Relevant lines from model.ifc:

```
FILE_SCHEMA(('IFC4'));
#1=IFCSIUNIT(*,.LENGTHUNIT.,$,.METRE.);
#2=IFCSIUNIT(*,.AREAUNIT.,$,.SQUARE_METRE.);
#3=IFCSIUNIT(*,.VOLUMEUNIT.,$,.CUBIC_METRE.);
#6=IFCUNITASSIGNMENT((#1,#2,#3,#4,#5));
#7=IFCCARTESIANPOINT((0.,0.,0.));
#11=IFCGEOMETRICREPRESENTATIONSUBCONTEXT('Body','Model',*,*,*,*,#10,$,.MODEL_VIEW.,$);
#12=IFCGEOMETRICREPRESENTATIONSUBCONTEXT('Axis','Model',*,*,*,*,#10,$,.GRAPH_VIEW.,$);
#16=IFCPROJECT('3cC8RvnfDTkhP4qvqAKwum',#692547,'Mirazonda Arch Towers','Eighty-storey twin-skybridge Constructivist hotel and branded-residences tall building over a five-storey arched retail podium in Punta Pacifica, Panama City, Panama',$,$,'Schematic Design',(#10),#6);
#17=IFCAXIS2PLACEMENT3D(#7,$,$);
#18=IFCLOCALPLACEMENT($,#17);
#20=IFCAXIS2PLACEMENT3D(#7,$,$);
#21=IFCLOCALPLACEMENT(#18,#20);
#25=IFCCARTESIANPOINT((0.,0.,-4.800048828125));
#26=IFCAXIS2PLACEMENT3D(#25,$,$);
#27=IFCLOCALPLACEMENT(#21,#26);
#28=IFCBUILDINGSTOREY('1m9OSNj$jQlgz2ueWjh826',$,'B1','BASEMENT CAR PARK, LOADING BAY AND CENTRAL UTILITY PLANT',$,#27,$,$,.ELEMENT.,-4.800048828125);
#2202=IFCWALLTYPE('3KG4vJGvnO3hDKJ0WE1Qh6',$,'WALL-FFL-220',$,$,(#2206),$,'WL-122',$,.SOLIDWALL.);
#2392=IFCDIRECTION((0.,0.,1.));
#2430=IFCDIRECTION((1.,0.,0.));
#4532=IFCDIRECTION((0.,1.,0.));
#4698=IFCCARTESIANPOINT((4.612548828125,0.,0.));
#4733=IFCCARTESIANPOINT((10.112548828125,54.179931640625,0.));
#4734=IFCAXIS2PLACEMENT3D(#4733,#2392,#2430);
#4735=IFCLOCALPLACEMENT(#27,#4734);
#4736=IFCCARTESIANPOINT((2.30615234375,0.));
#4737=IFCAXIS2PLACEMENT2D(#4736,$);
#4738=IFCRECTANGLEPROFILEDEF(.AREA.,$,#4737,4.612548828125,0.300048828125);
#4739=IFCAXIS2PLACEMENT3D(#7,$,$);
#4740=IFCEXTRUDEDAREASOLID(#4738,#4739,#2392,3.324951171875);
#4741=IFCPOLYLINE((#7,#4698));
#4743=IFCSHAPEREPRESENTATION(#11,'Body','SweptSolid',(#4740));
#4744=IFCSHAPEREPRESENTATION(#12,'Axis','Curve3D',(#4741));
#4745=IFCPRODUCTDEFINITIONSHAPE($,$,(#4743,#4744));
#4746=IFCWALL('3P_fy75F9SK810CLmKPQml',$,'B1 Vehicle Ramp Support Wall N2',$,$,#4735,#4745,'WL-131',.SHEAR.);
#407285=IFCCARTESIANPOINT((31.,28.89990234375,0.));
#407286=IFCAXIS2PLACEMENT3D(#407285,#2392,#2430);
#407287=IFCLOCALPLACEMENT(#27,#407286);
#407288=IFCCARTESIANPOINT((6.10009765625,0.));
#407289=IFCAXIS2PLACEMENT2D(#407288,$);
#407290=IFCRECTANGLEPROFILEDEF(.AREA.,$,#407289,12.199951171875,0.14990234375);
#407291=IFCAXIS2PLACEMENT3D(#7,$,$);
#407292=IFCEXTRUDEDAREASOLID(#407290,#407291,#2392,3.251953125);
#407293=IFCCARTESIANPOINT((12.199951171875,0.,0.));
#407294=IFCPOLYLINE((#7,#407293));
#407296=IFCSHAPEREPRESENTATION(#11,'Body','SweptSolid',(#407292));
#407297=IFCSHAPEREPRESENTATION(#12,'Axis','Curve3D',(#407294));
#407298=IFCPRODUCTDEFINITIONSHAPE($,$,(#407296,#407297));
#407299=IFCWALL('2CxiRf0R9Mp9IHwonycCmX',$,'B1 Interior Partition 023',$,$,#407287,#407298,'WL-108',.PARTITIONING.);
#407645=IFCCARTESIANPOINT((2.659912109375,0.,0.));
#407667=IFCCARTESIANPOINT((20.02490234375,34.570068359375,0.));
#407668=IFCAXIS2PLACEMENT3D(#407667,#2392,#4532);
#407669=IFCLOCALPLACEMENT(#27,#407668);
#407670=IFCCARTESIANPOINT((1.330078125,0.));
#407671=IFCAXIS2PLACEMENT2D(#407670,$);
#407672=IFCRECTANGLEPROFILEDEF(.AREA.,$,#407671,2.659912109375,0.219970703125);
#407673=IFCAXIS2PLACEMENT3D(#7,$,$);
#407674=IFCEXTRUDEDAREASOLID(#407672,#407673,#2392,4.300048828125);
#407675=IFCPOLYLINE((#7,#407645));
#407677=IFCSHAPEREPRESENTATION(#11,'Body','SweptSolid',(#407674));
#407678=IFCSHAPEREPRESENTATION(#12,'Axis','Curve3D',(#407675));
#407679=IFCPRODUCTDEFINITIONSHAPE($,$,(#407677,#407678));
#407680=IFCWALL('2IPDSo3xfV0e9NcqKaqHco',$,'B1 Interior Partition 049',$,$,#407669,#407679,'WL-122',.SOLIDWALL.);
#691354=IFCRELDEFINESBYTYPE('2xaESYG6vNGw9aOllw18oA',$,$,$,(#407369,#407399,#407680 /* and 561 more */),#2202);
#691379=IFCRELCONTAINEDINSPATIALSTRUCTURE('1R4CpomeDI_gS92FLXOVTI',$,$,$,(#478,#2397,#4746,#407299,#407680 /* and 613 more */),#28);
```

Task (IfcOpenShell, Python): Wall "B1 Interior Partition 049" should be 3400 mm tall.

```python
import ifcopenshell
import ifcopenshell.geom
import ifcopenshell.util.representation
import ifcopenshell.util.shape
import ifcopenshell.util.unit

model = ifcopenshell.open("model.ifc")
unit_scale = ifcopenshell.util.unit.calculate_unit_scale(model)
settings = ifcopenshell.geom.settings()


def volume(element):
    """Net volume in cubic metres, openings subtracted."""
    shape = ifcopenshell.geom.create_shape(settings, element)
    return ifcopenshell.util.shape.get_volume(shape.geometry)


wall = model.by_id(407680)
before = volume(wall)

body = ifcopenshell.util.representation.get_representation(wall, "Model", "Body")
solid = body.Items[0]
old_height = solid.Depth
solid.Depth = 3.4 / unit_scale
after = volume(wall)

print(f"height {old_height:g} -> {solid.Depth:g}, volume {before:.3f} -> {after:.3f} m3")

model.write("model_updated.ifc")
```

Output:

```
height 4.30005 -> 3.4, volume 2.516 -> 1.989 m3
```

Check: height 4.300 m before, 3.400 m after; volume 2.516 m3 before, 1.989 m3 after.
